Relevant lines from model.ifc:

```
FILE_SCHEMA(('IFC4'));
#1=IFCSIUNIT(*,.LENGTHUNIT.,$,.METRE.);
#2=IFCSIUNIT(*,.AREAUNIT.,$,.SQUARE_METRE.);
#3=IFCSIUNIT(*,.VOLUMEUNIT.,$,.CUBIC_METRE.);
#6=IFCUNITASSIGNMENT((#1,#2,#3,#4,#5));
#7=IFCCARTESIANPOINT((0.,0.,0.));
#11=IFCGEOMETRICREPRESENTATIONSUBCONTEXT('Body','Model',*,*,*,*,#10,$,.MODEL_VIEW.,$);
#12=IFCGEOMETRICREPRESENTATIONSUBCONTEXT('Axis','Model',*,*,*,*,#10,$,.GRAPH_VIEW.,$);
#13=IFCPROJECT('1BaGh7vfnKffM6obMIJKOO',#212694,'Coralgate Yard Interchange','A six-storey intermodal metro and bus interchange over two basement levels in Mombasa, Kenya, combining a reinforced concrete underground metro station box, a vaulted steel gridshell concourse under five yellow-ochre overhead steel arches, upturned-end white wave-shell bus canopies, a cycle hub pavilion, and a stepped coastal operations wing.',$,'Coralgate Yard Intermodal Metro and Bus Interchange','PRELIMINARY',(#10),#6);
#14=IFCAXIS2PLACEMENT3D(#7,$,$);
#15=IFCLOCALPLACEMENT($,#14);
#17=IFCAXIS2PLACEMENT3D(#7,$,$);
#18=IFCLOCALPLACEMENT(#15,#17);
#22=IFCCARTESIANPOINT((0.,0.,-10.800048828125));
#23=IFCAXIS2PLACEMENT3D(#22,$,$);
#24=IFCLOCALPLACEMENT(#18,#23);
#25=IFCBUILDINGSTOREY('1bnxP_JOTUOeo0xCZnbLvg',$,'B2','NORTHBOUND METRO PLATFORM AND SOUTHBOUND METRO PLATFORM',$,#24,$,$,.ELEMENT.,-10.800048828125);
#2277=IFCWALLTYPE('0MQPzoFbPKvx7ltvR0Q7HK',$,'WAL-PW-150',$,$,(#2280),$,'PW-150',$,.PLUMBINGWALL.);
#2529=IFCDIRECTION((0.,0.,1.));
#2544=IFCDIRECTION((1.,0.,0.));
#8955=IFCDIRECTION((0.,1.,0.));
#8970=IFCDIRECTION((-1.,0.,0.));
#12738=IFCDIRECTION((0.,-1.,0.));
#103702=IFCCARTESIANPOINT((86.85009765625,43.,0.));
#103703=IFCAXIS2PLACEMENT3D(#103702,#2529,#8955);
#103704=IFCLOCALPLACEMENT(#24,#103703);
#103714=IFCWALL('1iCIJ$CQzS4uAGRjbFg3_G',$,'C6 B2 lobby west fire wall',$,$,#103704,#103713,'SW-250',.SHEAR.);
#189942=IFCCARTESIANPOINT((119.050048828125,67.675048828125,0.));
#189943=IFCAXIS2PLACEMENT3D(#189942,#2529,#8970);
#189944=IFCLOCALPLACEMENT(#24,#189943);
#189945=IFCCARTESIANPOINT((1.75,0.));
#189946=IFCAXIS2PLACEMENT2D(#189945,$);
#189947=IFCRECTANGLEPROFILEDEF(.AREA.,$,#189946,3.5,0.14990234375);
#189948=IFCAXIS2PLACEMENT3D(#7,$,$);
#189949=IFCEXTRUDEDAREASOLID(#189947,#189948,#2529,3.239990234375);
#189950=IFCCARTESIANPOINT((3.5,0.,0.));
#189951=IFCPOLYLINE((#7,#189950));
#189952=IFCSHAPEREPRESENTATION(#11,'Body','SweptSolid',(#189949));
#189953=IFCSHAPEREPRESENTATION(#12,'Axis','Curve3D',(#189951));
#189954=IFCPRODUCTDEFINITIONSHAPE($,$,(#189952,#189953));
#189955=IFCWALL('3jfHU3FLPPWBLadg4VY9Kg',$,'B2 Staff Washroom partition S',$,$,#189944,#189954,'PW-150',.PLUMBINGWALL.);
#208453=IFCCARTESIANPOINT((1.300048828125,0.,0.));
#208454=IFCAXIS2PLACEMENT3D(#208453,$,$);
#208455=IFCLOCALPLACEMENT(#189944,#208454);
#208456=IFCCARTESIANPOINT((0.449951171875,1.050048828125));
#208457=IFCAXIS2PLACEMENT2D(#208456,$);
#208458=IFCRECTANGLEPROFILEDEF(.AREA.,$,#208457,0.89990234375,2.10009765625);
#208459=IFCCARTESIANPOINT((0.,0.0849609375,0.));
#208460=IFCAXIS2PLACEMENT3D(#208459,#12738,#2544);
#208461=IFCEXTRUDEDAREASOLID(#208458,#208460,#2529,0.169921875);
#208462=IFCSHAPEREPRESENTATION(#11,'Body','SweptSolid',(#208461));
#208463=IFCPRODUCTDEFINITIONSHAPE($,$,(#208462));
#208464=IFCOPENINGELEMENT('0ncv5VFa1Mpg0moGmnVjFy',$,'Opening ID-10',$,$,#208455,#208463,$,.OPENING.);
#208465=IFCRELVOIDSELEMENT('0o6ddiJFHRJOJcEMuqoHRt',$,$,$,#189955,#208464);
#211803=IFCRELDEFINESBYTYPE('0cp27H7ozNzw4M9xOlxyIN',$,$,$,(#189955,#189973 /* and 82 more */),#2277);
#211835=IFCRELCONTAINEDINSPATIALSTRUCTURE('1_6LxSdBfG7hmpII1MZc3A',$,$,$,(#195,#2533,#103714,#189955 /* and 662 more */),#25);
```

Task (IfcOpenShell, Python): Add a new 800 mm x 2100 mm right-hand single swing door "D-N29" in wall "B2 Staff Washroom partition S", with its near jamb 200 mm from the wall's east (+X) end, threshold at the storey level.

```python
import numpy as np
import ifcopenshell
import ifcopenshell.api.feature
import ifcopenshell.api.geometry
import ifcopenshell.api.root
import ifcopenshell.api.spatial
import ifcopenshell.geom
import ifcopenshell.util.element
import ifcopenshell.util.placement
import ifcopenshell.util.representation
import ifcopenshell.util.shape
import ifcopenshell.util.unit

model = ifcopenshell.open("model.ifc")
unit_scale = ifcopenshell.util.unit.calculate_unit_scale(model)
settings = ifcopenshell.geom.settings()


def volume(element):
    """Net volume in cubic metres, openings subtracted."""
    shape = ifcopenshell.geom.create_shape(settings, element)
    return ifcopenshell.util.shape.get_volume(shape.geometry)


wall = model.by_guid("3jfHU3FLPPWBLadg4VY9Kg")
storey = ifcopenshell.util.element.get_container(wall, ifc_class="IfcBuildingStorey")
context = ifcopenshell.util.representation.get_context(model, "Model", "Body", "MODEL_VIEW")
before = volume(wall)

width, height, from_end, sill = 0.8, 2.1, 0.2, 0.0  # metres

# The wall runs along its own X axis, and the end named is its -X end.
wall_shape = ifcopenshell.geom.create_shape(settings, wall)
x, y, z = ifcopenshell.util.shape.get_vertices(wall_shape.geometry).T
start = x.min() + from_end
face, thickness = float(y.min()), float(y.max() - y.min())
wall_matrix = ifcopenshell.util.placement.get_local_placement(wall.ObjectPlacement)
level = ifcopenshell.util.placement.get_local_placement(storey.ObjectPlacement)[2, 3]


def in_wall(x, y):
    """Placement at x, y metres in the wall's axes, at sill height."""
    matrix = wall_matrix.copy()
    matrix[:, 3] = wall_matrix @ np.array([x / unit_scale, y / unit_scale, 0.0, 1.0])
    matrix[2, 3] = level + sill / unit_scale
    return matrix


# Opening: a box that overshoots both wall faces by 50 mm.
opening = ifcopenshell.api.root.create_entity(model, ifc_class="IfcOpeningElement", predefined_type="OPENING")
box = ifcopenshell.api.geometry.add_wall_representation(
    model, context=context, length=width, height=height, thickness=thickness + 0.1
)
ifcopenshell.api.geometry.assign_representation(model, product=opening, representation=box)
ifcopenshell.api.geometry.edit_object_placement(model, product=opening, matrix=in_wall(start, face - 0.05), is_si=False)
ifcopenshell.api.feature.add_feature(model, feature=opening, element=wall)

door = ifcopenshell.api.root.create_entity(model, ifc_class="IfcDoor", name="D-N29", predefined_type="DOOR")
door.OverallWidth, door.OverallHeight = width / unit_scale, height / unit_scale
door.OperationType = "SINGLE_SWING_RIGHT"
body = ifcopenshell.api.geometry.add_door_representation(
    model,
    context=context,
    overall_width=door.OverallWidth,
    overall_height=door.OverallHeight,
    operation_type="SINGLE_SWING_RIGHT",
    lining_properties={"LiningDepth": thickness / unit_scale, "ThresholdDepth": thickness / unit_scale},
)
ifcopenshell.api.geometry.assign_representation(model, product=door, representation=body)
ifcopenshell.api.spatial.assign_container(model, products=[door], relating_structure=storey)
ifcopenshell.api.feature.add_filling(model, opening=opening, element=door)

# The lining spans the wall, so the door starts at the wall face.
ifcopenshell.api.geometry.edit_object_placement(model, product=door, matrix=in_wall(start, face), is_si=False)

after = volume(wall)

print(f"wall volume {before:.3f} -> {after:.3f} m3")

model.write("model_edited.ifc")
```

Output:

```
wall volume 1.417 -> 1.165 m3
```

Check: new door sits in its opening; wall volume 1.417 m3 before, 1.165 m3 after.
